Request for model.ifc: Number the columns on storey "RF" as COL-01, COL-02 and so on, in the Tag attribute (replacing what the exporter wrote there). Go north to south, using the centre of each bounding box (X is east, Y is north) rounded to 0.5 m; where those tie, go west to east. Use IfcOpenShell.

First a look at what the model holds.

```python
import ifcopenshell
import ifcopenshell.util.element
import ifcopenshell.util.placement

model = ifcopenshell.open("model.ifc")
print(model.schema)
storey = next(s for s in model.by_type("IfcBuildingStorey") if s.Name == "RF")
columns = [e for e in ifcopenshell.util.element.get_decomposition(storey) if e.is_a("IfcColumn")]
for e in sorted(columns, key=lambda e: e.id()):
    origin = ifcopenshell.util.placement.get_local_placement(e.ObjectPlacement)[:3, 3]
    print(e.id(), e.Tag, e.Name, origin.round(2) + 0.0, sep=" | ")
```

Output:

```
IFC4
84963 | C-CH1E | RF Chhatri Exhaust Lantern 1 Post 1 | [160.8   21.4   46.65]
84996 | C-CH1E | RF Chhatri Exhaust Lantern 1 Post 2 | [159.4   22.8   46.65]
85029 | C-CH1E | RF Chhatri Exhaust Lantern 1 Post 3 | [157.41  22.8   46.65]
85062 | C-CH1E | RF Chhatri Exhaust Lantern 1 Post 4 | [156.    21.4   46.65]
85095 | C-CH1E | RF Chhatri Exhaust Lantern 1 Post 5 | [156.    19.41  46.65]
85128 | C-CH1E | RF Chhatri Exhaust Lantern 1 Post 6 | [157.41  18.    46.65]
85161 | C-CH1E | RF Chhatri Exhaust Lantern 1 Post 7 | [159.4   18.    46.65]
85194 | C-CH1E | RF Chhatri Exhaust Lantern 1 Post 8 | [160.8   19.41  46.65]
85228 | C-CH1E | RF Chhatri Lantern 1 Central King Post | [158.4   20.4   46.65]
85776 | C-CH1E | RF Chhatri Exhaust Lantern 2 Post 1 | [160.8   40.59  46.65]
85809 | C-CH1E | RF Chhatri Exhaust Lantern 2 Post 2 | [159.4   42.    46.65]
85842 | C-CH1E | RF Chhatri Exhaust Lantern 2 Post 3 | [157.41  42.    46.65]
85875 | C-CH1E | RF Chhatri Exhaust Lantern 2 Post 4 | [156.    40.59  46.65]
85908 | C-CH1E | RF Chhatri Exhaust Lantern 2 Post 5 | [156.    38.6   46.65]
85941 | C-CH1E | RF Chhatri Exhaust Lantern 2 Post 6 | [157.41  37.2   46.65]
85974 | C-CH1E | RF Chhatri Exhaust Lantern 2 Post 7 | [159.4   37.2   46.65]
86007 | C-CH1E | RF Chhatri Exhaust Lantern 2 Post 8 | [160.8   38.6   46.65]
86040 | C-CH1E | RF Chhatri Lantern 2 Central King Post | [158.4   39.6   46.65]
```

```python
import ifcopenshell
import ifcopenshell.geom
import ifcopenshell.util.element
import ifcopenshell.util.shape

model = ifcopenshell.open("model.ifc")
settings = ifcopenshell.geom.settings()
settings.set("use-world-coords", True)


def centre(element):
    shape = ifcopenshell.geom.create_shape(settings, element)
    return ifcopenshell.util.shape.get_bbox_centroid(shape.geometry)


storey = next(s for s in model.by_type("IfcBuildingStorey") if s.Name == "RF")
columns = [e for e in ifcopenshell.util.element.get_decomposition(storey) if e.is_a("IfcColumn")]

# Insertion points can sit at a corner or the storey origin, so sort by the geometry (in metres).
centres = {e: centre(e) for e in columns}
columns.sort(key=lambda e: (-round(centres[e][1] / 0.5), centres[e][0]))

for i, e in enumerate(columns, start=1):
    number = f"COL-{i:02d}"
    e.Tag = number
    print(e.id(), number)

model.write("model_rev.ifc")
```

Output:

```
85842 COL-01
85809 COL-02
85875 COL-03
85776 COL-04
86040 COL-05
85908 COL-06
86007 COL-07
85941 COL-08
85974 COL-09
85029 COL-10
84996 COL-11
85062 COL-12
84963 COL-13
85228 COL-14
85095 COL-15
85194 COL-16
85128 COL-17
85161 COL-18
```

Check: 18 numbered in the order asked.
